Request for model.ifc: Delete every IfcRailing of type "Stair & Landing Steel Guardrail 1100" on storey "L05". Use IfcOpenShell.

First a look at what the model holds.

```python
import ifcopenshell
import ifcopenshell.util.element

model = ifcopenshell.open("model.ifc")
print(model.schema)
storey = next(s for s in model.by_type("IfcBuildingStorey") if s.Name == "L05")
railings = [e for e in ifcopenshell.util.element.get_decomposition(storey) if e.is_a("IfcRailing")]
seen = {}
for e in railings:
    element_type = ifcopenshell.util.element.get_type(e)
    name = element_type.Name if element_type not in (None, e) else None
    seen[name] = seen.get(name, 0) + 1
for name, count in sorted(seen.items(), key=str):
    print(count, "x", name)
```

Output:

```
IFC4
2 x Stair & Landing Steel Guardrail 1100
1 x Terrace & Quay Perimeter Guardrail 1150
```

```python
import ifcopenshell
import ifcopenshell.api.root
import ifcopenshell.util.element

model = ifcopenshell.open("model.ifc")

storey = next(s for s in model.by_type("IfcBuildingStorey") if s.Name == "L05")
railings = [e for e in ifcopenshell.util.element.get_decomposition(storey) if e.is_a("IfcRailing")]
targets = [e for e in railings if (t := ifcopenshell.util.element.get_type(e)) not in (None, e) and t.Name == "Stair & Landing Steel Guardrail 1100"]

for e in targets:
    ifcopenshell.api.root.remove_product(model, product=e)
print(len(targets), "removed")

model.write("model-out.ifc")
```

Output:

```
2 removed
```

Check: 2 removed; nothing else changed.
